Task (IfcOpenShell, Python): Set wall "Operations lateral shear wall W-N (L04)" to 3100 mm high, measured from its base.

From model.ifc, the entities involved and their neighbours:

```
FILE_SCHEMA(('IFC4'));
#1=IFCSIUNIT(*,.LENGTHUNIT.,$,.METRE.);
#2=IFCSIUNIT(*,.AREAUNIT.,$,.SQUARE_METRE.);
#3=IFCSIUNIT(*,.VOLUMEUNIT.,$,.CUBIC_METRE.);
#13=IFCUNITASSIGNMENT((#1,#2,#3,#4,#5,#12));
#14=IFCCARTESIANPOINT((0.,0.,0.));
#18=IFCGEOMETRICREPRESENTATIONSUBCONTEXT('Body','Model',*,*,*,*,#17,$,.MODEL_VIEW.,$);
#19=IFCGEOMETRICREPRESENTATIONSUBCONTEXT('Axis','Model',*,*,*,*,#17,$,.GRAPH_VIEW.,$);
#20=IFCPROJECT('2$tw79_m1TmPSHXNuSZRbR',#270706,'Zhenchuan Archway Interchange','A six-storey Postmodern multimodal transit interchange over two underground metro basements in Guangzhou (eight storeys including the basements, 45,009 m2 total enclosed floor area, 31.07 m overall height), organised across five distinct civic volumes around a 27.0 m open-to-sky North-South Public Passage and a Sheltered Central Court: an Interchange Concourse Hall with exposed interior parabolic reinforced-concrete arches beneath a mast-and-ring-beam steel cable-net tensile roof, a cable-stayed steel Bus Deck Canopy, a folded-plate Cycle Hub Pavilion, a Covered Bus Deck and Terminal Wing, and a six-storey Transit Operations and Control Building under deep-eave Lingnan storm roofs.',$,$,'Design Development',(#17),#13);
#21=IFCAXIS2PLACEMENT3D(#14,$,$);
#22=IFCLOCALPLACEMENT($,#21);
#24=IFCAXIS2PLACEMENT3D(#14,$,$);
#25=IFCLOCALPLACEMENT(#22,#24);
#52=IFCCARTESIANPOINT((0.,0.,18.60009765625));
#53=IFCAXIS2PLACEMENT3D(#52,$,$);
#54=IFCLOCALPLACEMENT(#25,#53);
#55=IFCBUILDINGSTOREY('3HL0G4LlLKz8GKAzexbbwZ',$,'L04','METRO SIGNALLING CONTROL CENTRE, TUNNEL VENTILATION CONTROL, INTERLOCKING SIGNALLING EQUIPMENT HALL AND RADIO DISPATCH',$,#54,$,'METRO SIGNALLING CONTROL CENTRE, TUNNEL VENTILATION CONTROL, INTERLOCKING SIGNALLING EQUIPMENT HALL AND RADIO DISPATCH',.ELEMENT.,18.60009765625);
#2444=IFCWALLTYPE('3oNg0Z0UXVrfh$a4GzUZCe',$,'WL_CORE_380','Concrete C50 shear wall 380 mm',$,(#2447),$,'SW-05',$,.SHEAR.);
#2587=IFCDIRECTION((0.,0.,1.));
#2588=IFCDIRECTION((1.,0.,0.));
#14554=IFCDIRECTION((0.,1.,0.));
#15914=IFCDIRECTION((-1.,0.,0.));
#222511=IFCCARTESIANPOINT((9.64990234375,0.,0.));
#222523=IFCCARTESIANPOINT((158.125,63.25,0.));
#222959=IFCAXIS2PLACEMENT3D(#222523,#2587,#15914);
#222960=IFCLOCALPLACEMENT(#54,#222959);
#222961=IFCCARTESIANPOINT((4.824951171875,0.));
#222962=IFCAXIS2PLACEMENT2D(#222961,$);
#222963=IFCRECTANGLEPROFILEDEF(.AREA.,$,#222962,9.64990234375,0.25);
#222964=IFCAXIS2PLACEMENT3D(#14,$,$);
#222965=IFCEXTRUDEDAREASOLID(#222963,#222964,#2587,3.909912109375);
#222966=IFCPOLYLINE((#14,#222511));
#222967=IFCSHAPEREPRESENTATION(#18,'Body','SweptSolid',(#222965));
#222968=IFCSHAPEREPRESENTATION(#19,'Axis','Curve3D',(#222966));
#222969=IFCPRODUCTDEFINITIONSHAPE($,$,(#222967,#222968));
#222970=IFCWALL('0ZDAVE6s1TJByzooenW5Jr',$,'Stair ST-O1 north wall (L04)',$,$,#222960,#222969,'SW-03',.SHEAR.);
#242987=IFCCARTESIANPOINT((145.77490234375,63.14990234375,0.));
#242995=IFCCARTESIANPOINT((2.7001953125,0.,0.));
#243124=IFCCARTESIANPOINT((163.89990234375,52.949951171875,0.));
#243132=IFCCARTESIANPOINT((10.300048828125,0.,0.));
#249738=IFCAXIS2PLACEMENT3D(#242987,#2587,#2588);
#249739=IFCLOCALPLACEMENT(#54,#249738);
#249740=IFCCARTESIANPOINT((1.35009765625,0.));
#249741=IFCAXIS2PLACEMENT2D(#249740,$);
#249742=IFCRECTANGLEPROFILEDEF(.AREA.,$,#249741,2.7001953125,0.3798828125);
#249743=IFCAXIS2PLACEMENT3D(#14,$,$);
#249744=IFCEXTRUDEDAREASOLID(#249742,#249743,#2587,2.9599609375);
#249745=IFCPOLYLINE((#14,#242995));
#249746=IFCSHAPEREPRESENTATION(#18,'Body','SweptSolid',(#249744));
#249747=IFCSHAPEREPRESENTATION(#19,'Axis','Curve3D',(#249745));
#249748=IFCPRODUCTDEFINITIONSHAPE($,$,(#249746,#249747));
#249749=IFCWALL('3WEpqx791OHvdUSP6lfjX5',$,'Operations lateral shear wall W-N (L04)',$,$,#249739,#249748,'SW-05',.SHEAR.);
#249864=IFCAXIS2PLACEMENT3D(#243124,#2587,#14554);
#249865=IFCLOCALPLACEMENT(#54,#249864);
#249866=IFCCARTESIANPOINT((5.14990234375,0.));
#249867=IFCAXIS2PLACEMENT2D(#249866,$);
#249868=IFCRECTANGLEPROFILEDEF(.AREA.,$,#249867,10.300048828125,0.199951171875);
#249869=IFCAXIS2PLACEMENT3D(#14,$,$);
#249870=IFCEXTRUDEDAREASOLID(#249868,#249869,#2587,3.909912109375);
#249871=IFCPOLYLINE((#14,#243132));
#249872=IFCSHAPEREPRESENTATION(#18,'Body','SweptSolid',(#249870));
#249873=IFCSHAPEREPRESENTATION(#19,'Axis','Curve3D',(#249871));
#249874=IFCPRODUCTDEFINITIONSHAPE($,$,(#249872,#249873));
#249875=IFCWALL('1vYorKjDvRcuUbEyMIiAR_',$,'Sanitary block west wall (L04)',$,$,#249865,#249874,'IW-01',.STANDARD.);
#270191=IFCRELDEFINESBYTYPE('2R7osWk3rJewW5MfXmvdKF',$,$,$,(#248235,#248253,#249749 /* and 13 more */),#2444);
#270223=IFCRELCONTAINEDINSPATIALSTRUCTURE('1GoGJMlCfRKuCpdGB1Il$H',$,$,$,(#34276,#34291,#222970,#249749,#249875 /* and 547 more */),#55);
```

```python
import ifcopenshell
import ifcopenshell.geom
import ifcopenshell.util.representation
import ifcopenshell.util.shape

model = ifcopenshell.open("model.ifc")
settings = ifcopenshell.geom.settings()


def volume(element):
    """Net volume in cubic metres, openings subtracted."""
    shape = ifcopenshell.geom.create_shape(settings, element)
    return ifcopenshell.util.shape.get_volume(shape.geometry)


wall = model.by_id(249749)
before = volume(wall)

body = ifcopenshell.util.representation.get_representation(wall, "Model", "Body")
solid = body.Items[0]
old_height = solid.Depth
solid.Depth = 3.1
after = volume(wall)

print(f"height {old_height:g} -> {solid.Depth:g}, volume {before:.3f} -> {after:.3f} m3")

model.write("model_rev.ifc")
```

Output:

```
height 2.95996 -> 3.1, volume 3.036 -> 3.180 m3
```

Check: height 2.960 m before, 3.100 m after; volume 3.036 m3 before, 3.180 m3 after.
